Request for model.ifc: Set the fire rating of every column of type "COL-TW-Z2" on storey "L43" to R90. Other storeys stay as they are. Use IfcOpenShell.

First a look at what the model holds.

```python
import ifcopenshell
import ifcopenshell.util.element

model = ifcopenshell.open("model.ifc")
print(model.schema)
storey = next(s for s in model.by_type("IfcBuildingStorey") if s.Name == "L43")
columns = [e for e in ifcopenshell.util.element.get_decomposition(storey) if e.is_a("IfcColumn")]
seen = {}
for e in columns:
    element_type = ifcopenshell.util.element.get_type(e)
    key = (element_type.Name if element_type != e and element_type else None, ifcopenshell.util.element.get_pset(e, "Pset_ColumnCommon", "FireRating"))
    seen[key] = seen.get(key, 0) + 1
for (name, value), count in sorted(seen.items(), key=str):
    print(count, "x", name, "|", value)
```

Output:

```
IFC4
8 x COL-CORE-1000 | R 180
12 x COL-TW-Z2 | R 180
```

```python
import ifcopenshell
import ifcopenshell.api.pset
import ifcopenshell.util.element

model = ifcopenshell.open("model.ifc")

storey = next(s for s in model.by_type("IfcBuildingStorey") if s.Name == "L43")
columns = [e for e in ifcopenshell.util.element.get_decomposition(storey) if e.is_a("IfcColumn")]

count = 0
for e in columns:
    element_type = ifcopenshell.util.element.get_type(e)
    if element_type in (None, e) or element_type.Name != "COL-TW-Z2":
        continue
    found = ifcopenshell.util.element.get_pset(e, "Pset_ColumnCommon", should_inherit=False)
    if found:
        pset = model.by_id(found["id"])
        if len(ifcopenshell.util.element.get_elements_by_pset(pset)) > 1:
            pset = ifcopenshell.api.pset.unshare_pset(model, products=[e], pset=pset)[0]
    else:
        pset = ifcopenshell.api.pset.add_pset(model, product=e, name="Pset_ColumnCommon")
    ifcopenshell.api.pset.edit_pset(model, pset=pset, properties={"FireRating": "R90"})
    count += 1

print(count, "columns updated")

model.write("model_updated.ifc")
```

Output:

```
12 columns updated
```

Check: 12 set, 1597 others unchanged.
